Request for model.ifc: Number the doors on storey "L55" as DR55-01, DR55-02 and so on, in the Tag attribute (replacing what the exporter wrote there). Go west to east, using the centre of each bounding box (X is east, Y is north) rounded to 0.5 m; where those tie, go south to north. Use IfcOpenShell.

First a look at what the model holds.

```python
import ifcopenshell
import ifcopenshell.util.element
import ifcopenshell.util.placement

model = ifcopenshell.open("model.ifc")
print(model.schema)
storey = next(s for s in model.by_type("IfcBuildingStorey") if s.Name == "L55")
doors = [e for e in ifcopenshell.util.element.get_decomposition(storey) if e.is_a("IfcDoor")]
for e in sorted(doors, key=lambda e: e.id()):
    origin = ifcopenshell.util.placement.get_local_placement(e.ObjectPlacement)[:3, 3]
    print(e.id(), e.Tag, e.Name, origin.round(2) + 0.0, sep=" | ")
```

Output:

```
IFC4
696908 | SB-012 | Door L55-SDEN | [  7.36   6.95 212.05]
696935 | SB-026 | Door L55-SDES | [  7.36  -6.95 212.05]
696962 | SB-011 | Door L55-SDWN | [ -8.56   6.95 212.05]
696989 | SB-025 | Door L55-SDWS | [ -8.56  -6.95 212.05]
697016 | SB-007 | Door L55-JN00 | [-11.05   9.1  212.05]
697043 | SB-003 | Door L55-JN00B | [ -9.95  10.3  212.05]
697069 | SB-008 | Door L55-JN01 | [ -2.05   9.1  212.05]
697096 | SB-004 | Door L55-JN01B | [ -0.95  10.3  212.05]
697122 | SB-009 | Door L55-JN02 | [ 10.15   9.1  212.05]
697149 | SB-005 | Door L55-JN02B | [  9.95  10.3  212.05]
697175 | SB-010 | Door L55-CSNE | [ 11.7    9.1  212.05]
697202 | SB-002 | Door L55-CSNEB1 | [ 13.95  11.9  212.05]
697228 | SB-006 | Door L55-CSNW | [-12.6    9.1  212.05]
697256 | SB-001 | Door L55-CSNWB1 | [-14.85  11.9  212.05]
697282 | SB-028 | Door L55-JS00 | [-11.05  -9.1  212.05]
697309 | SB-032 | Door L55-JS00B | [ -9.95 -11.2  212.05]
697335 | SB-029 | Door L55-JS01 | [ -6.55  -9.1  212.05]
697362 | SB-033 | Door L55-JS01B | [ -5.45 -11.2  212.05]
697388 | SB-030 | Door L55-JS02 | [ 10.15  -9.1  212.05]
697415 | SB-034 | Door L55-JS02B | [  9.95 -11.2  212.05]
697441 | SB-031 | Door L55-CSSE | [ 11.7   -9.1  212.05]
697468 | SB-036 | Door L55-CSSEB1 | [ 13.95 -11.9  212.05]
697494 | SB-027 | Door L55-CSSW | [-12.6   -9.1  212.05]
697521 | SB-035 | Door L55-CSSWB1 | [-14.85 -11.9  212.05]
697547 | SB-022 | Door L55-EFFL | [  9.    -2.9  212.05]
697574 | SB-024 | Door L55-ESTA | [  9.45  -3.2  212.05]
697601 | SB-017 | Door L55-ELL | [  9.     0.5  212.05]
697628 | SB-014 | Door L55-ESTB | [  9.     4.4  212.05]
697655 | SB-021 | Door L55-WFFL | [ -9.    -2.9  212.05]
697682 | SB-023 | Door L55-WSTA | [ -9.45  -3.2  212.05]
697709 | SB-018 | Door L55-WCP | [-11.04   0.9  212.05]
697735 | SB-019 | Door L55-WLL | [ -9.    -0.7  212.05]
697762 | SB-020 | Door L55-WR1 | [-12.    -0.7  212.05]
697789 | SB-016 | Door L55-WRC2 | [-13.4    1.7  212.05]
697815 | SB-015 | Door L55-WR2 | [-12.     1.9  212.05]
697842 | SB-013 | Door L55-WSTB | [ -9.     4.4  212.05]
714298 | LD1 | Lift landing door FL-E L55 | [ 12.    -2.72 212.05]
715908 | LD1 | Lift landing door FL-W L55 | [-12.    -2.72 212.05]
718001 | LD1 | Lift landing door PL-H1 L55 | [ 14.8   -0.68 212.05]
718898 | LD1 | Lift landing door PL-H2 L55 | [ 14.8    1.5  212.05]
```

```python
import ifcopenshell
import ifcopenshell.geom
import ifcopenshell.util.element
import ifcopenshell.util.shape

model = ifcopenshell.open("model.ifc")
settings = ifcopenshell.geom.settings()
settings.set("use-world-coords", True)


def centre(element):
    shape = ifcopenshell.geom.create_shape(settings, element)
    return ifcopenshell.util.shape.get_bbox_centroid(shape.geometry)


storey = next(s for s in model.by_type("IfcBuildingStorey") if s.Name == "L55")
doors = [e for e in ifcopenshell.util.element.get_decomposition(storey) if e.is_a("IfcDoor")]

# Insertion points can sit at a corner or the storey origin, so sort by the geometry (in metres).
centres = {e: centre(e) for e in doors}
doors.sort(key=lambda e: (round(centres[e][0] / 0.5), centres[e][1]))

for i, e in enumerate(doors, start=1):
    number = f"DR55-{i:02d}"
    e.Tag = number
    print(e.id(), number)

model.write("model_edited.ifc")
```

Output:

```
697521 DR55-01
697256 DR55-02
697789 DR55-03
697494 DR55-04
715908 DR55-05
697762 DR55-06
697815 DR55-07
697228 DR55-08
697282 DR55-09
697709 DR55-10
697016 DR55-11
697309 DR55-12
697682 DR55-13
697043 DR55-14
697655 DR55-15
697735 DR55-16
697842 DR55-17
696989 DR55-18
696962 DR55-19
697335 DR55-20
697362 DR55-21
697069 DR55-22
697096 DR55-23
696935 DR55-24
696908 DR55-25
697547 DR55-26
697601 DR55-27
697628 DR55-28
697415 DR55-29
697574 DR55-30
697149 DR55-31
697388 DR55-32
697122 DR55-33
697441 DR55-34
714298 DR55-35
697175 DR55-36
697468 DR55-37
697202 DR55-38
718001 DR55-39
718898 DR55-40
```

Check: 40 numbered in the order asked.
